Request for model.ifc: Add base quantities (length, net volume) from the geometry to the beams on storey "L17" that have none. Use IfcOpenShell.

First a look at what the model holds.

```python
import ifcopenshell
import ifcopenshell.util.element
import ifcopenshell.util.unit

model = ifcopenshell.open("model.ifc")
print(model.schema)
for unit_type in ("LENGTHUNIT", "AREAUNIT", "VOLUMEUNIT"):
    print(unit_type, ifcopenshell.util.unit.calculate_unit_scale(model, unit_type))
storey = next(s for s in model.by_type("IfcBuildingStorey") if s.Name == "L17")
beams = [e for e in ifcopenshell.util.element.get_decomposition(storey) if e.is_a("IfcBeam")]
for e in sorted(beams, key=lambda e: e.id()):
    print(e.id(), e.is_a(), e.Name, list(ifcopenshell.util.element.get_psets(e, qtos_only=True)), sep=" | ")
```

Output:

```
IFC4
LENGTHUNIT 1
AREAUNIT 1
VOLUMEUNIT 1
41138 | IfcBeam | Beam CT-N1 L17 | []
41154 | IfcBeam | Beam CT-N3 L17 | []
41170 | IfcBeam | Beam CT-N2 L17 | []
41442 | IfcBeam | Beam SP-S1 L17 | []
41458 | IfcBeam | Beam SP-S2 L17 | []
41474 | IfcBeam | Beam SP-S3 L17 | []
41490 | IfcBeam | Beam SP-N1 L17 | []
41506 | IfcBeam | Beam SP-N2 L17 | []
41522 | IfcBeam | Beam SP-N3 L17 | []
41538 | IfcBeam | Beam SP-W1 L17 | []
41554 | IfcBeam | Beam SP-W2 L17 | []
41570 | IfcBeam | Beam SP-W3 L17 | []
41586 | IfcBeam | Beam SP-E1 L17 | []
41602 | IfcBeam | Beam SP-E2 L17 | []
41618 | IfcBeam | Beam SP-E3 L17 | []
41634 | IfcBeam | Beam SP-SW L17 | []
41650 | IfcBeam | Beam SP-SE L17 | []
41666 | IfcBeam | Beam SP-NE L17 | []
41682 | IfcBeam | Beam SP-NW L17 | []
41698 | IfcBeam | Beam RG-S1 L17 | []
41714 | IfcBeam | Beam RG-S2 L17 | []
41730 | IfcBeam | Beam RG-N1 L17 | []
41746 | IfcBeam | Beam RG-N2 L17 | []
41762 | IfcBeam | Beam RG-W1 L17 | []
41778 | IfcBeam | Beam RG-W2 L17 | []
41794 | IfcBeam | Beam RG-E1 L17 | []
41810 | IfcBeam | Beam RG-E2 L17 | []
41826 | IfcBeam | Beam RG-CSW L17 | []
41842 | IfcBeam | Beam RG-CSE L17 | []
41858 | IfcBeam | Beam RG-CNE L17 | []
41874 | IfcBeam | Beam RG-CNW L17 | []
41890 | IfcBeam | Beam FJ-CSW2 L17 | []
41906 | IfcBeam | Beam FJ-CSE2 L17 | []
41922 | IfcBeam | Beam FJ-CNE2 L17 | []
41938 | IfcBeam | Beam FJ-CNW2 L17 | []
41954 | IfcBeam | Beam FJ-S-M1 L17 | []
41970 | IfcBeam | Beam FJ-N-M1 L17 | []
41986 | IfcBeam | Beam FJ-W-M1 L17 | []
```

```python
import ifcopenshell
import ifcopenshell.api.pset
import ifcopenshell.geom
import ifcopenshell.util.element
import ifcopenshell.util.shape
import ifcopenshell.util.unit

model = ifcopenshell.open("model.ifc")
unit_scale = ifcopenshell.util.unit.calculate_unit_scale(model)
volume_scale = ifcopenshell.util.unit.calculate_unit_scale(model, "VOLUMEUNIT")
settings = ifcopenshell.geom.settings()

storey = next(s for s in model.by_type("IfcBuildingStorey") if s.Name == "L17")
beams = [e for e in ifcopenshell.util.element.get_decomposition(storey) if e.is_a("IfcBeam")]

for e in sorted(beams, key=lambda e: e.id()):
    if ifcopenshell.util.element.get_psets(e, qtos_only=True, should_inherit=False):
        continue
    # Geometry comes back in metres, in the element's own axes.
    shape = ifcopenshell.geom.create_shape(settings, e)
    values = {
        "Length": ifcopenshell.util.shape.get_max_xyz(shape.geometry) / unit_scale,
        "NetVolume": ifcopenshell.util.shape.get_volume(shape.geometry) / volume_scale,
    }
    qto = ifcopenshell.api.pset.add_qto(model, product=e, name="Qto_BeamBaseQuantities")
    ifcopenshell.api.pset.edit_qto(model, qto=qto, properties=values)
    print(e.id(), {k: round(v, 3) for k, v in values.items()})

model.write("model-out.ifc")
```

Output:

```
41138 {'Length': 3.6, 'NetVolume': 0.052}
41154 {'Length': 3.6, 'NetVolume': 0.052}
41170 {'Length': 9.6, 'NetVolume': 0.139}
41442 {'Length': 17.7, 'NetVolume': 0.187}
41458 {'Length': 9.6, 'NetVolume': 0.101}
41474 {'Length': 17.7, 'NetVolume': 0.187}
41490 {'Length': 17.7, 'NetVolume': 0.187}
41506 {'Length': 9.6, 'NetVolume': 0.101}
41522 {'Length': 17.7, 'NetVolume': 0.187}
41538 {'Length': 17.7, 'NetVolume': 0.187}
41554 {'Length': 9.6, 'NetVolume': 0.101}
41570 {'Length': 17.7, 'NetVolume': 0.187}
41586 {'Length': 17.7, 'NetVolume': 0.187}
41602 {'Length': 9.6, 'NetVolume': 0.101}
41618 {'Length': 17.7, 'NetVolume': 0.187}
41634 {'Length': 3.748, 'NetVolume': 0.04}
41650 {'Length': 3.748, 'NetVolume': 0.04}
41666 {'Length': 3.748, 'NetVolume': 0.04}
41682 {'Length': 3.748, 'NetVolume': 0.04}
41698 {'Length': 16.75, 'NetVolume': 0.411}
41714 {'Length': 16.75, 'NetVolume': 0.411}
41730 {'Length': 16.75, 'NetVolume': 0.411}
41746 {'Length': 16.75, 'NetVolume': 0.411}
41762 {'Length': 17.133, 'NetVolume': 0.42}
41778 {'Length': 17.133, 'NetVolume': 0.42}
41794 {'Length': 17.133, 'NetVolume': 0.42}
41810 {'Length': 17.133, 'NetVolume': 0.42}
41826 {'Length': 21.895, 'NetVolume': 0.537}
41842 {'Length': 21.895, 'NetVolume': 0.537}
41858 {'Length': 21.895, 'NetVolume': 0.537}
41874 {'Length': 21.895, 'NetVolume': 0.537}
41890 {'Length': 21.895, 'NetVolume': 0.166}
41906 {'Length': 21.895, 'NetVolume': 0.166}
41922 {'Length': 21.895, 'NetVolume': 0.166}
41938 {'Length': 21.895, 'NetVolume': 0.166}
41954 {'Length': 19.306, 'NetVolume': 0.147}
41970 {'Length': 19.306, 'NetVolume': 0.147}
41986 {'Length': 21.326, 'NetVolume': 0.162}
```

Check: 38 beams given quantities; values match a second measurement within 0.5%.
